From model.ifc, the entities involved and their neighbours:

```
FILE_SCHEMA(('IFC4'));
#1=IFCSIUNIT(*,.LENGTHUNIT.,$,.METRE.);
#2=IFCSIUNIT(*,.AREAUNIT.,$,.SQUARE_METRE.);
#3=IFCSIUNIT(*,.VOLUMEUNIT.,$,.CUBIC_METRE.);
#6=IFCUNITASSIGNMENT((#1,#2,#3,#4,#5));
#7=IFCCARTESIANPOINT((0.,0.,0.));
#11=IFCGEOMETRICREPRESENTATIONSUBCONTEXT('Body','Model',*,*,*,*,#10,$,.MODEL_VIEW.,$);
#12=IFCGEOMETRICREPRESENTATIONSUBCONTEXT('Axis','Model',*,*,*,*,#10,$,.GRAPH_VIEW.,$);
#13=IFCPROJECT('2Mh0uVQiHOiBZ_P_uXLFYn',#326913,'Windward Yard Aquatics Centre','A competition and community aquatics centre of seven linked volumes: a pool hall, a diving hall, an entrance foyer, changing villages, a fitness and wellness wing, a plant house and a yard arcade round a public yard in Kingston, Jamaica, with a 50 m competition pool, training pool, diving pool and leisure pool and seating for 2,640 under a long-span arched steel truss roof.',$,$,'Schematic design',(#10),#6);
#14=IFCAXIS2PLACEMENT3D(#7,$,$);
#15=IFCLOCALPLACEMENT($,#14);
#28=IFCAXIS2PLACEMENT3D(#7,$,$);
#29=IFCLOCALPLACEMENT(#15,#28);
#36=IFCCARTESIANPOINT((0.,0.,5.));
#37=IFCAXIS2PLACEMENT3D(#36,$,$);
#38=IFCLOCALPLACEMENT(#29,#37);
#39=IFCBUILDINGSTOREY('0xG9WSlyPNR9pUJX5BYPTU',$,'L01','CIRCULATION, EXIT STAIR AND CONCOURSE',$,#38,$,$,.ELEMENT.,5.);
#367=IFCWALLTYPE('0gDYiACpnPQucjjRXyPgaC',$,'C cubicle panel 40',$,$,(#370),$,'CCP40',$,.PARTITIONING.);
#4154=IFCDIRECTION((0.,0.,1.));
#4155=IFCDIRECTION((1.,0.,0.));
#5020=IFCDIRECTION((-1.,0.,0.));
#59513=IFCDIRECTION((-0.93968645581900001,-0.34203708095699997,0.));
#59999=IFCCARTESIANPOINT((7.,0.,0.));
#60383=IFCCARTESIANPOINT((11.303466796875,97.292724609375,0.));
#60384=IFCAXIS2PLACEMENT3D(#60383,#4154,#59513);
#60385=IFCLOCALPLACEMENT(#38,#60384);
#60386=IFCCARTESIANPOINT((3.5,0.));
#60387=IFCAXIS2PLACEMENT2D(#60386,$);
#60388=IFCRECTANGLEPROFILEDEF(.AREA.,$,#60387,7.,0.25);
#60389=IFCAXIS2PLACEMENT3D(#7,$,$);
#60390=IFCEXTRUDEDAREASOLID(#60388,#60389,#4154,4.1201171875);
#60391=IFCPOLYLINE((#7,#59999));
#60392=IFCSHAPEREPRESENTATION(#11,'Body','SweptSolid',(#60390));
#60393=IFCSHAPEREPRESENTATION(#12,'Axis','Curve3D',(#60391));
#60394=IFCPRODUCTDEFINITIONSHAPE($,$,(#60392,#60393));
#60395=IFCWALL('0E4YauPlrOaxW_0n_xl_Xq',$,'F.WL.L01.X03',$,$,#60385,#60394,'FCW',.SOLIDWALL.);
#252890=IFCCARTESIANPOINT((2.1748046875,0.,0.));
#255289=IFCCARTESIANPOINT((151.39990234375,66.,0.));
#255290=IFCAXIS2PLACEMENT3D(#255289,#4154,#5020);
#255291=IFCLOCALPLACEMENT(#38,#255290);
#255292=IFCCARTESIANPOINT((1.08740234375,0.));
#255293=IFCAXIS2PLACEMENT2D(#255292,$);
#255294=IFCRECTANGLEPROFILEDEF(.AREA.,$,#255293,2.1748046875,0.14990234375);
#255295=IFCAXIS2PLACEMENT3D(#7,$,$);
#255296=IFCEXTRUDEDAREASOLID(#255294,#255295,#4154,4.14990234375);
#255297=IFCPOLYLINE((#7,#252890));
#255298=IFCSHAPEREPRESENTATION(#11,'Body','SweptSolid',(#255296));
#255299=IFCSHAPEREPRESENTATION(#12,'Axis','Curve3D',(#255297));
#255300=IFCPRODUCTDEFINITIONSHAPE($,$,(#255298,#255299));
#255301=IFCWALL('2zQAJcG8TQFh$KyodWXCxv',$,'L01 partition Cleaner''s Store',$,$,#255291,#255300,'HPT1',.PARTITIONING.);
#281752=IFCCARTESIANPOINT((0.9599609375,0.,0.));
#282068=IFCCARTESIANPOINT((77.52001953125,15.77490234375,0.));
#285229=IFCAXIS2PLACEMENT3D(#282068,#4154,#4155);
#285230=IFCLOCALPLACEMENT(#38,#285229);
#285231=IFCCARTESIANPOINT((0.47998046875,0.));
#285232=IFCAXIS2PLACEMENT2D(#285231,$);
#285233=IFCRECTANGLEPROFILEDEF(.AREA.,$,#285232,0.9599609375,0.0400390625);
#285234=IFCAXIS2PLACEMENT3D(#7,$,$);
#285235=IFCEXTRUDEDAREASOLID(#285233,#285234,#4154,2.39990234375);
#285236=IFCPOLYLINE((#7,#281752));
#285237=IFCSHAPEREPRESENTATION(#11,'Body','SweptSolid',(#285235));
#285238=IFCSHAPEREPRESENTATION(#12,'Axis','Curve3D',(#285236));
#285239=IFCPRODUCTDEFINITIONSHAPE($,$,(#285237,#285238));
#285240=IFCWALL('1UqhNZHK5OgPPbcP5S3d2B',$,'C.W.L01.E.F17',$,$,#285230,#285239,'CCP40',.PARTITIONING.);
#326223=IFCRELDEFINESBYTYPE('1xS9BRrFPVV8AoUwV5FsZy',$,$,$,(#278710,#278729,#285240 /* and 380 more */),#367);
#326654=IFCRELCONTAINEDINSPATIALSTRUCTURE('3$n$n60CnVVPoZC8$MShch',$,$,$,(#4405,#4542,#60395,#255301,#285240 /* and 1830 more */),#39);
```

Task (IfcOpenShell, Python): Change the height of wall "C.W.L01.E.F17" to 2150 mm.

```python
import ifcopenshell
import ifcopenshell.geom
import ifcopenshell.util.representation
import ifcopenshell.util.shape

model = ifcopenshell.open("model.ifc")
settings = ifcopenshell.geom.settings()


def volume(element):
    """Net volume in cubic metres, openings subtracted."""
    shape = ifcopenshell.geom.create_shape(settings, element)
    return ifcopenshell.util.shape.get_volume(shape.geometry)


wall = model.by_guid("1UqhNZHK5OgPPbcP5S3d2B")
before = volume(wall)

body = ifcopenshell.util.representation.get_representation(wall, "Model", "Body")
solid = body.Items[0]
old_height = solid.Depth
solid.Depth = 2.15
after = volume(wall)

print(f"height {old_height:g} -> {solid.Depth:g}, volume {before:.3f} -> {after:.3f} m3")

model.write("model_rev.ifc")
```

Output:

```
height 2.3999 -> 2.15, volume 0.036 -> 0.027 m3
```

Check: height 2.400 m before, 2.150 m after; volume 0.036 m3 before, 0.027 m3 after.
